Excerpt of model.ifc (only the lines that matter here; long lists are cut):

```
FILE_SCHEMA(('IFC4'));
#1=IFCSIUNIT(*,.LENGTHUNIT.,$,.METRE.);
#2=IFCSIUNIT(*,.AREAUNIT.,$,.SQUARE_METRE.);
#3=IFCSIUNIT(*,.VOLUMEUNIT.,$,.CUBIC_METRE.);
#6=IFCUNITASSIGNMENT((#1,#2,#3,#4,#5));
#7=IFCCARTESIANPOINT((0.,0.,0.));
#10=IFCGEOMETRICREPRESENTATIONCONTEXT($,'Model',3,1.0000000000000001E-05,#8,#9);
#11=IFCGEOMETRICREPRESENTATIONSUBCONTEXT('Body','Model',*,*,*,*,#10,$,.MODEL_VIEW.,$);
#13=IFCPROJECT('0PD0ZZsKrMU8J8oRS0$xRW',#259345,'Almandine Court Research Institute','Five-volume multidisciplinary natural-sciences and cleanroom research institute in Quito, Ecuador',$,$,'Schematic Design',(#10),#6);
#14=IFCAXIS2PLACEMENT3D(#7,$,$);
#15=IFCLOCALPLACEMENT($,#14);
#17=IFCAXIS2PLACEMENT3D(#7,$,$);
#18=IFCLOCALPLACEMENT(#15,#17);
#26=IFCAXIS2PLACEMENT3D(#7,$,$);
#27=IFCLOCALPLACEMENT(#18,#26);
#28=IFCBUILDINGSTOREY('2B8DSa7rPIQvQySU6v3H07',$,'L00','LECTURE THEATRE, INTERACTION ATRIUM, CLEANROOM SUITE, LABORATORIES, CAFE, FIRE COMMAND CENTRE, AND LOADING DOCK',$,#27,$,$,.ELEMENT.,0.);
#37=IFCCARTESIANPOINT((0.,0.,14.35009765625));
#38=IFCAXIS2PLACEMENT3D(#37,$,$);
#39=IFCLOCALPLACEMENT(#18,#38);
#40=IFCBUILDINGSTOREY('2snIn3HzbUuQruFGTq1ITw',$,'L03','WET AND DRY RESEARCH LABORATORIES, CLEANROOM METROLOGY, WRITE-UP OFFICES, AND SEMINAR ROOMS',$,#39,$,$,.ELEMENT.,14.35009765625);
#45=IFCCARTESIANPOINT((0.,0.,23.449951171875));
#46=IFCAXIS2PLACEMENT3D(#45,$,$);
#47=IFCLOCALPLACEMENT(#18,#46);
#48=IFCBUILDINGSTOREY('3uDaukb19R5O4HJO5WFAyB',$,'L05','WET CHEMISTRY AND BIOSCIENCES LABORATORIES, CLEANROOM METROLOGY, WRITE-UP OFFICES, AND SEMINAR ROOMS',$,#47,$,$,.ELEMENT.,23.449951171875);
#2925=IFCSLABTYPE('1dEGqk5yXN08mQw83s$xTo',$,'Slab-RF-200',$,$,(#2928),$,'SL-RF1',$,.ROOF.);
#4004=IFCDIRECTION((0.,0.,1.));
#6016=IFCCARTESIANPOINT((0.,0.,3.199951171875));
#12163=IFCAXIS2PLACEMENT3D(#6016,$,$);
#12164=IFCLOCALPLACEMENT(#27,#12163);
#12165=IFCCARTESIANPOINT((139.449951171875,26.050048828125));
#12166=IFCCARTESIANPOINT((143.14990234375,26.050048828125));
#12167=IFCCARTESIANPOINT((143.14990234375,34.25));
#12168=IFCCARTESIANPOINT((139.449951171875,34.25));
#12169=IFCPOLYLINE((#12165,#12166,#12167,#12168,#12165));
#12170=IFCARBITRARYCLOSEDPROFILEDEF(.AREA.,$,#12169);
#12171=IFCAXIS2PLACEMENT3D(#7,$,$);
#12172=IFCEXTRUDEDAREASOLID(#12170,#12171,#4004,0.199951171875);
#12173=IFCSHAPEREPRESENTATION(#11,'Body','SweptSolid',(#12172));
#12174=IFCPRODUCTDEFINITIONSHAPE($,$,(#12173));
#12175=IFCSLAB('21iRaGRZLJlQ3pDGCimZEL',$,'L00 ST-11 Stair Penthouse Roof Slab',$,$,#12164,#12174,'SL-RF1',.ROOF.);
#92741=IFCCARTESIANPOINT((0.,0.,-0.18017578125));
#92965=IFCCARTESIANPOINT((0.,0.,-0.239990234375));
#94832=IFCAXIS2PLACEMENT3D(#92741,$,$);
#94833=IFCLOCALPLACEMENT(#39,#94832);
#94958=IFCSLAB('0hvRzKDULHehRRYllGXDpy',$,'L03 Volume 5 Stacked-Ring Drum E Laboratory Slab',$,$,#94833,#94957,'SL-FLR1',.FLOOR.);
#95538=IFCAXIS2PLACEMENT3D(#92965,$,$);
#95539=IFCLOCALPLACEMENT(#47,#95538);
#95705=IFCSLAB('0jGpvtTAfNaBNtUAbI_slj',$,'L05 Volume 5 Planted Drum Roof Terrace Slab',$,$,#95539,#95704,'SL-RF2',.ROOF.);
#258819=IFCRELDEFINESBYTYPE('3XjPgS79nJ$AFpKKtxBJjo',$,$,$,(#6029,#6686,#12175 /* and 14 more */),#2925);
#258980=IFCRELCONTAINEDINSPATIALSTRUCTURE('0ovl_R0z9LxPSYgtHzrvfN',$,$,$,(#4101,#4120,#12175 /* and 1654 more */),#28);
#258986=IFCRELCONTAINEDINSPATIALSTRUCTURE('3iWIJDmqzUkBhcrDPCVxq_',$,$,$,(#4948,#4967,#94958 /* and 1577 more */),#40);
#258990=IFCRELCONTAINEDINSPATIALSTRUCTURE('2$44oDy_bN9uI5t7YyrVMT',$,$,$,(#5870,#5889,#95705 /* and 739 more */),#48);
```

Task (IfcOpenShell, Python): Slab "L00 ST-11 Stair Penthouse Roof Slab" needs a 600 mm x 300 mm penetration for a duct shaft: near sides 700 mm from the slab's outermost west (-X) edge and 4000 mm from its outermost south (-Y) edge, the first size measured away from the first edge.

```python
import numpy as np
import ifcopenshell
import ifcopenshell.api.feature
import ifcopenshell.api.geometry
import ifcopenshell.api.root
import ifcopenshell.geom
import ifcopenshell.util.placement
import ifcopenshell.util.representation
import ifcopenshell.util.shape
import ifcopenshell.util.unit

model = ifcopenshell.open("model.ifc")
unit_scale = ifcopenshell.util.unit.calculate_unit_scale(model)
settings = ifcopenshell.geom.settings()


def volume(element):
    """Net volume in cubic metres, openings subtracted."""
    shape = ifcopenshell.geom.create_shape(settings, element)
    return ifcopenshell.util.shape.get_volume(shape.geometry)


slab = model.by_guid("21iRaGRZLJlQ3pDGCimZEL")
before = volume(slab)

# Extent in the slab's own axes, in metres. The edges named are its -X and -Y sides.
slab_shape = ifcopenshell.geom.create_shape(settings, slab)
vertices = ifcopenshell.util.shape.get_vertices(slab_shape.geometry)
x_min, y_min, bottom = vertices.min(axis=0)
top = vertices[:, 2].max()

opening = ifcopenshell.api.root.create_entity(model, ifc_class="IfcOpeningElement", name="Duct shaft opening", predefined_type="OPENING")
context = ifcopenshell.util.representation.get_context(model, "Model", "Body", "MODEL_VIEW")
width, depth = 0.6, 0.3
outline = [(0.0, 0.0), (width, 0.0), (width, depth), (0.0, depth), (0.0, 0.0)]
# Overshoot both faces by 50 mm so the cut is clean.
shape = ifcopenshell.api.geometry.add_slab_representation(
    model, context=context, depth=top - bottom + 0.1, polyline=outline
)
ifcopenshell.api.geometry.assign_representation(model, product=opening, representation=shape)

matrix = ifcopenshell.util.placement.get_local_placement(slab.ObjectPlacement)
matrix[:, 3] = matrix @ np.append(np.array([x_min + 0.7, y_min + 4, bottom - 0.05]) / unit_scale, 1.0)
ifcopenshell.api.geometry.edit_object_placement(model, product=opening, matrix=matrix, is_si=False)
ifcopenshell.api.feature.add_feature(model, feature=opening, element=slab)

after = volume(slab)

print(f"slab volume {before:.3f} -> {after:.3f} m3")

model.write("model_rev.ifc")
```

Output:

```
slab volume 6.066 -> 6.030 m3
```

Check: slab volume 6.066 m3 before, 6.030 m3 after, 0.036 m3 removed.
